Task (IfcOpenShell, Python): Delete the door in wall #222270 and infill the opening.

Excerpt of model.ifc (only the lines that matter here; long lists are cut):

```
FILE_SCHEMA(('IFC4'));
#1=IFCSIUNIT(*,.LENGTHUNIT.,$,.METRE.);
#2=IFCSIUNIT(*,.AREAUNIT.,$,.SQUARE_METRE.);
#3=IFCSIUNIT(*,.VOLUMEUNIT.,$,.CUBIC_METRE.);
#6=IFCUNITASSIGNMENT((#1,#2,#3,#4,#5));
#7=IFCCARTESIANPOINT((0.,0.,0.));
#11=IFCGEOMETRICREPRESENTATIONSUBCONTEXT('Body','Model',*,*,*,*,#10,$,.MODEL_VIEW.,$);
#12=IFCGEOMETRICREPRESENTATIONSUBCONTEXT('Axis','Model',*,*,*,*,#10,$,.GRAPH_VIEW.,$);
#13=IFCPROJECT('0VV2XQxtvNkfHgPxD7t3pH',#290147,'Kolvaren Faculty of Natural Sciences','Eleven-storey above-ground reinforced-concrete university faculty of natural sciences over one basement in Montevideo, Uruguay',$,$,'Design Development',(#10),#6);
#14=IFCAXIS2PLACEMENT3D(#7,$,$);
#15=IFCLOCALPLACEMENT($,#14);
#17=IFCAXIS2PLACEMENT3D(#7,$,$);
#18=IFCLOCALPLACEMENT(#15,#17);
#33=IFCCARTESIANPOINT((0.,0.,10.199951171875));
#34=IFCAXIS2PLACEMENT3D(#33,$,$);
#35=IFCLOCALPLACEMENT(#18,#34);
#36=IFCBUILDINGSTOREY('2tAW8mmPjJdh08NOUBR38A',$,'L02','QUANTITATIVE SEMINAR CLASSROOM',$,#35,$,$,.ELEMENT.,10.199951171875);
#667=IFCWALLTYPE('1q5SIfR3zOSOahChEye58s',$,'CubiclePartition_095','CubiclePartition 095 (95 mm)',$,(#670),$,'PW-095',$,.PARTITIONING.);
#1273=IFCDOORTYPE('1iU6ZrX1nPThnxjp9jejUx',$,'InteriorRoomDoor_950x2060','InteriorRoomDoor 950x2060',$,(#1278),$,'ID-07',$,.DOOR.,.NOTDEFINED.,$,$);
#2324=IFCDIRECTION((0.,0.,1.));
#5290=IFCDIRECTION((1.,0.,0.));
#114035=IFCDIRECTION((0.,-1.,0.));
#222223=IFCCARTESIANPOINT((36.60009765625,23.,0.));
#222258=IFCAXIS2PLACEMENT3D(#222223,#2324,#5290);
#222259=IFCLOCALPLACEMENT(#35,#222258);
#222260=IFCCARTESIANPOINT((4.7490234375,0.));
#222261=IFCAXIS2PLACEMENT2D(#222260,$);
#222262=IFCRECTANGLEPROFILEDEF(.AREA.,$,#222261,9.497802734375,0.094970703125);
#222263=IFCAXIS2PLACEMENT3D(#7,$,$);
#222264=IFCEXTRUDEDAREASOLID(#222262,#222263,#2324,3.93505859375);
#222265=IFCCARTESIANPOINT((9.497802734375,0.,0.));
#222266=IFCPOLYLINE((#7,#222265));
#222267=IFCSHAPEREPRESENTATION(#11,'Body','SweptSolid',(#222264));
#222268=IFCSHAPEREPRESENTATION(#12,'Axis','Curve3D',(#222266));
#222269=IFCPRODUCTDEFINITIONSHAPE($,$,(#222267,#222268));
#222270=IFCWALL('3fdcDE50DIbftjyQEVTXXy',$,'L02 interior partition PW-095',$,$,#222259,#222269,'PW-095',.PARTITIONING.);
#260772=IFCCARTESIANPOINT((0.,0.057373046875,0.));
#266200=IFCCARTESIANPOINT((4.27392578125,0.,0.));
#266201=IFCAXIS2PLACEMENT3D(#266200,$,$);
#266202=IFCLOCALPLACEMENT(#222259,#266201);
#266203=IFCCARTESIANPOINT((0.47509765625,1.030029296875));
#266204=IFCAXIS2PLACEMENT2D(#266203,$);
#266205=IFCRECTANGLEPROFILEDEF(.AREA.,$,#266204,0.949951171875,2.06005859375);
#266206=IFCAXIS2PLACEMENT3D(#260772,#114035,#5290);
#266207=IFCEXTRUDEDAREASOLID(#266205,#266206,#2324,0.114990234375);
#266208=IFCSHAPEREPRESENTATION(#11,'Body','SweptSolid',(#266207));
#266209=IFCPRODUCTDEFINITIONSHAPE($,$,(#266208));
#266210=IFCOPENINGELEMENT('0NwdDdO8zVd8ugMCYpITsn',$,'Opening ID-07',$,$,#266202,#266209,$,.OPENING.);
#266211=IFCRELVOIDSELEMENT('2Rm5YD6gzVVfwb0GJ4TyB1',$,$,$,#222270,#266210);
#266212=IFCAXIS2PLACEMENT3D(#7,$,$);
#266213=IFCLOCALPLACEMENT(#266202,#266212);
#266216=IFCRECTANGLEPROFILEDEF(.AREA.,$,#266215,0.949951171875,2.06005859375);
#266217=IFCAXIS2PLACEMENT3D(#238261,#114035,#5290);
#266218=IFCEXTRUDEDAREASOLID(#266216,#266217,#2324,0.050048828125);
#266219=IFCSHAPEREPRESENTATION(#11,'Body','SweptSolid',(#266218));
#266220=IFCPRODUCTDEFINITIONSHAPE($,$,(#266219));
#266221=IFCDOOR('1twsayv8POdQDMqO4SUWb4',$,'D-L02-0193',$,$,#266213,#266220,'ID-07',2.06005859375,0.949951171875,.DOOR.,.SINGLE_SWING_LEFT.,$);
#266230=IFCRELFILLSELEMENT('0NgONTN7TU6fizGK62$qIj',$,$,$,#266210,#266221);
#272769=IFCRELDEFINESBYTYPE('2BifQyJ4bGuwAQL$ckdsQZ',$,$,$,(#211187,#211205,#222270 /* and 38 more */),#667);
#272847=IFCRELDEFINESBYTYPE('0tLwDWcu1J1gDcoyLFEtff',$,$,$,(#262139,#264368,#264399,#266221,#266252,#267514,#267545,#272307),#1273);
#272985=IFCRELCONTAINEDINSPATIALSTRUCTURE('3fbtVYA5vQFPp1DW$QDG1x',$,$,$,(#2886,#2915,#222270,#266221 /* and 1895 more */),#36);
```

```python
import ifcopenshell
import ifcopenshell.api.feature
import ifcopenshell.api.root
import ifcopenshell.geom
import ifcopenshell.util.shape

model = ifcopenshell.open("model.ifc")
settings = ifcopenshell.geom.settings()


def volume(element):
    """Net volume in cubic metres, openings subtracted."""
    shape = ifcopenshell.geom.create_shape(settings, element)
    return ifcopenshell.util.shape.get_volume(shape.geometry)


door = model.by_guid("1twsayv8POdQDMqO4SUWb4")
opening = door.FillsVoids[0].RelatingOpeningElement
wall = opening.VoidsElements[0].RelatingBuildingElement
before = volume(wall)

ifcopenshell.api.root.remove_product(model, product=door)
ifcopenshell.api.feature.remove_feature(model, feature=opening)

after = volume(wall)

print(f"wall volume {before:.3f} -> {after:.3f} m3")

model.write("model_edited.ifc")
```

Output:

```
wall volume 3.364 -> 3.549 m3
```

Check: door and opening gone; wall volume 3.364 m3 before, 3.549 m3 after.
